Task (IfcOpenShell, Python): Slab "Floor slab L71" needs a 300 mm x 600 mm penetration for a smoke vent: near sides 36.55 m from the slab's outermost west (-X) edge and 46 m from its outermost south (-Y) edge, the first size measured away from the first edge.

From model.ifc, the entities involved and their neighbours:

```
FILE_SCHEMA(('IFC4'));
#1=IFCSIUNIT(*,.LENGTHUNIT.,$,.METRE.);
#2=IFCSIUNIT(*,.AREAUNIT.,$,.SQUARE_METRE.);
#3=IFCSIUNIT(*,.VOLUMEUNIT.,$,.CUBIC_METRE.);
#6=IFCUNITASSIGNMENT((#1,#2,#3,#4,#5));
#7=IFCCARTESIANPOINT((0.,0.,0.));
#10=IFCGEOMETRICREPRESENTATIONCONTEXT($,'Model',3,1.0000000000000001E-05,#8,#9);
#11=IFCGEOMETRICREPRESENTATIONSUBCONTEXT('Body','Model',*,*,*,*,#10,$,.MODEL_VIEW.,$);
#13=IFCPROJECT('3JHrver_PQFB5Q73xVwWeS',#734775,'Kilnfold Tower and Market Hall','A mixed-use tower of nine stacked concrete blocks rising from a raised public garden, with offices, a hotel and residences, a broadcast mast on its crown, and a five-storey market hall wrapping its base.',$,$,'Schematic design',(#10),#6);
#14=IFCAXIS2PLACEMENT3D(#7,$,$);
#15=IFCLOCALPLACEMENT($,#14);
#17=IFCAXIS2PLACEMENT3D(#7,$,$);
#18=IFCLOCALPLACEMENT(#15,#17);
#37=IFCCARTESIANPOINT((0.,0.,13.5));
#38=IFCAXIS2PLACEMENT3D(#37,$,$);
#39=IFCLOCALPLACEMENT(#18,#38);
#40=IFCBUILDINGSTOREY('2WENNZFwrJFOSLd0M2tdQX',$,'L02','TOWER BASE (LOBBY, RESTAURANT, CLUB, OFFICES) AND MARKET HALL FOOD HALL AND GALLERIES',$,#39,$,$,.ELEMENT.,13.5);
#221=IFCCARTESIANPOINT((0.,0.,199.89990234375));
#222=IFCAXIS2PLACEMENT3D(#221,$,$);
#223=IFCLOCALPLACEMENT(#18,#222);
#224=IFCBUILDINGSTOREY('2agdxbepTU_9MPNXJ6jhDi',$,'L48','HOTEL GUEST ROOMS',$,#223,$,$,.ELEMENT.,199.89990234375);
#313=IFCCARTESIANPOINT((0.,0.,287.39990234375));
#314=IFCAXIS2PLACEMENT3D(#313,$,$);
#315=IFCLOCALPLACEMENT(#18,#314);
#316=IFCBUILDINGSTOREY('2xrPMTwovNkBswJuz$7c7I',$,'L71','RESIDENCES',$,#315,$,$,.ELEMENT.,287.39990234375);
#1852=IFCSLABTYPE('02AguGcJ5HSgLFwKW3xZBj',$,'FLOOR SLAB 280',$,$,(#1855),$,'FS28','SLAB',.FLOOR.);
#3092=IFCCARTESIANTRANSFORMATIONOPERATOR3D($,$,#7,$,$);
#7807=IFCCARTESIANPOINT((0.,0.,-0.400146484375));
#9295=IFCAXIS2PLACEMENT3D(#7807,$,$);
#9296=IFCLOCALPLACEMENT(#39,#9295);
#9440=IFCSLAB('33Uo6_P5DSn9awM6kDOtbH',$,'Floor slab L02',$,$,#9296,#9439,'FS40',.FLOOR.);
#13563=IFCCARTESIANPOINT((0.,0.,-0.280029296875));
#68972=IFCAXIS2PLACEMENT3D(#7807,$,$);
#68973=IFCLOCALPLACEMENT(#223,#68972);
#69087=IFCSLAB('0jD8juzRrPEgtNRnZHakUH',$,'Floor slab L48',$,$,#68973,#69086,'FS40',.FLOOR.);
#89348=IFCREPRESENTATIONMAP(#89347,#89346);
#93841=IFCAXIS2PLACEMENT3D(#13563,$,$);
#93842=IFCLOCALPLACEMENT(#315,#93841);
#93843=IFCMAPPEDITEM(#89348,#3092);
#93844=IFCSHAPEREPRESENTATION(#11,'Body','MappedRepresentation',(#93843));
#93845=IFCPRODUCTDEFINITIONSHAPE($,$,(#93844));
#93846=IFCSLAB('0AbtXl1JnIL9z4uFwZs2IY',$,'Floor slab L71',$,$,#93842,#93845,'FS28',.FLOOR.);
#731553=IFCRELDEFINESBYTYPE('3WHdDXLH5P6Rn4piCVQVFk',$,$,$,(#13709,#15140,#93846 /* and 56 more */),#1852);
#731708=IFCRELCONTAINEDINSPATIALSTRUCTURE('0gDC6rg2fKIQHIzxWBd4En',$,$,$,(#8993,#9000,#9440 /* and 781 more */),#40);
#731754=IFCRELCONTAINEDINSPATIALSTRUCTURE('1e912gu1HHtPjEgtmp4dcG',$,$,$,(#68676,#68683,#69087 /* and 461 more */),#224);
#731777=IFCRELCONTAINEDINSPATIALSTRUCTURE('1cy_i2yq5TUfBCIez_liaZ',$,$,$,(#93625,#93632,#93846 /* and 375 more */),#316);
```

```python
import numpy as np
import ifcopenshell
import ifcopenshell.api.feature
import ifcopenshell.api.geometry
import ifcopenshell.api.root
import ifcopenshell.geom
import ifcopenshell.util.placement
import ifcopenshell.util.representation
import ifcopenshell.util.shape
import ifcopenshell.util.unit

model = ifcopenshell.open("model.ifc")
unit_scale = ifcopenshell.util.unit.calculate_unit_scale(model)
settings = ifcopenshell.geom.settings()


def volume(element):
    """Net volume in cubic metres, openings subtracted."""
    shape = ifcopenshell.geom.create_shape(settings, element)
    return ifcopenshell.util.shape.get_volume(shape.geometry)


slab = model.by_id(93846)
before = volume(slab)

# Extent in the slab's own axes, in metres. The edges named are its -X and -Y sides.
slab_shape = ifcopenshell.geom.create_shape(settings, slab)
vertices = ifcopenshell.util.shape.get_vertices(slab_shape.geometry)
x_min, y_min, bottom = vertices.min(axis=0)
top = vertices[:, 2].max()

opening = ifcopenshell.api.root.create_entity(model, ifc_class="IfcOpeningElement", name="Smoke vent opening", predefined_type="OPENING")
context = ifcopenshell.util.representation.get_context(model, "Model", "Body", "MODEL_VIEW")
width, depth = 0.3, 0.6
outline = [(0.0, 0.0), (width, 0.0), (width, depth), (0.0, depth), (0.0, 0.0)]
# Overshoot both faces by 50 mm so the cut is clean.
shape = ifcopenshell.api.geometry.add_slab_representation(
    model, context=context, depth=top - bottom + 0.1, polyline=outline
)
ifcopenshell.api.geometry.assign_representation(model, product=opening, representation=shape)

matrix = ifcopenshell.util.placement.get_local_placement(slab.ObjectPlacement)
matrix[:, 3] = matrix @ np.append(np.array([x_min + 36.55, y_min + 46, bottom - 0.05]) / unit_scale, 1.0)
ifcopenshell.api.geometry.edit_object_placement(model, product=opening, matrix=matrix, is_si=False)
ifcopenshell.api.feature.add_feature(model, feature=opening, element=slab)

after = volume(slab)

print(f"slab volume {before:.3f} -> {after:.3f} m3")

model.write("model-out.ifc")
```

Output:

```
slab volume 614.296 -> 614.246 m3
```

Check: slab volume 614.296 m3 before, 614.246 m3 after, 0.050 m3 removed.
